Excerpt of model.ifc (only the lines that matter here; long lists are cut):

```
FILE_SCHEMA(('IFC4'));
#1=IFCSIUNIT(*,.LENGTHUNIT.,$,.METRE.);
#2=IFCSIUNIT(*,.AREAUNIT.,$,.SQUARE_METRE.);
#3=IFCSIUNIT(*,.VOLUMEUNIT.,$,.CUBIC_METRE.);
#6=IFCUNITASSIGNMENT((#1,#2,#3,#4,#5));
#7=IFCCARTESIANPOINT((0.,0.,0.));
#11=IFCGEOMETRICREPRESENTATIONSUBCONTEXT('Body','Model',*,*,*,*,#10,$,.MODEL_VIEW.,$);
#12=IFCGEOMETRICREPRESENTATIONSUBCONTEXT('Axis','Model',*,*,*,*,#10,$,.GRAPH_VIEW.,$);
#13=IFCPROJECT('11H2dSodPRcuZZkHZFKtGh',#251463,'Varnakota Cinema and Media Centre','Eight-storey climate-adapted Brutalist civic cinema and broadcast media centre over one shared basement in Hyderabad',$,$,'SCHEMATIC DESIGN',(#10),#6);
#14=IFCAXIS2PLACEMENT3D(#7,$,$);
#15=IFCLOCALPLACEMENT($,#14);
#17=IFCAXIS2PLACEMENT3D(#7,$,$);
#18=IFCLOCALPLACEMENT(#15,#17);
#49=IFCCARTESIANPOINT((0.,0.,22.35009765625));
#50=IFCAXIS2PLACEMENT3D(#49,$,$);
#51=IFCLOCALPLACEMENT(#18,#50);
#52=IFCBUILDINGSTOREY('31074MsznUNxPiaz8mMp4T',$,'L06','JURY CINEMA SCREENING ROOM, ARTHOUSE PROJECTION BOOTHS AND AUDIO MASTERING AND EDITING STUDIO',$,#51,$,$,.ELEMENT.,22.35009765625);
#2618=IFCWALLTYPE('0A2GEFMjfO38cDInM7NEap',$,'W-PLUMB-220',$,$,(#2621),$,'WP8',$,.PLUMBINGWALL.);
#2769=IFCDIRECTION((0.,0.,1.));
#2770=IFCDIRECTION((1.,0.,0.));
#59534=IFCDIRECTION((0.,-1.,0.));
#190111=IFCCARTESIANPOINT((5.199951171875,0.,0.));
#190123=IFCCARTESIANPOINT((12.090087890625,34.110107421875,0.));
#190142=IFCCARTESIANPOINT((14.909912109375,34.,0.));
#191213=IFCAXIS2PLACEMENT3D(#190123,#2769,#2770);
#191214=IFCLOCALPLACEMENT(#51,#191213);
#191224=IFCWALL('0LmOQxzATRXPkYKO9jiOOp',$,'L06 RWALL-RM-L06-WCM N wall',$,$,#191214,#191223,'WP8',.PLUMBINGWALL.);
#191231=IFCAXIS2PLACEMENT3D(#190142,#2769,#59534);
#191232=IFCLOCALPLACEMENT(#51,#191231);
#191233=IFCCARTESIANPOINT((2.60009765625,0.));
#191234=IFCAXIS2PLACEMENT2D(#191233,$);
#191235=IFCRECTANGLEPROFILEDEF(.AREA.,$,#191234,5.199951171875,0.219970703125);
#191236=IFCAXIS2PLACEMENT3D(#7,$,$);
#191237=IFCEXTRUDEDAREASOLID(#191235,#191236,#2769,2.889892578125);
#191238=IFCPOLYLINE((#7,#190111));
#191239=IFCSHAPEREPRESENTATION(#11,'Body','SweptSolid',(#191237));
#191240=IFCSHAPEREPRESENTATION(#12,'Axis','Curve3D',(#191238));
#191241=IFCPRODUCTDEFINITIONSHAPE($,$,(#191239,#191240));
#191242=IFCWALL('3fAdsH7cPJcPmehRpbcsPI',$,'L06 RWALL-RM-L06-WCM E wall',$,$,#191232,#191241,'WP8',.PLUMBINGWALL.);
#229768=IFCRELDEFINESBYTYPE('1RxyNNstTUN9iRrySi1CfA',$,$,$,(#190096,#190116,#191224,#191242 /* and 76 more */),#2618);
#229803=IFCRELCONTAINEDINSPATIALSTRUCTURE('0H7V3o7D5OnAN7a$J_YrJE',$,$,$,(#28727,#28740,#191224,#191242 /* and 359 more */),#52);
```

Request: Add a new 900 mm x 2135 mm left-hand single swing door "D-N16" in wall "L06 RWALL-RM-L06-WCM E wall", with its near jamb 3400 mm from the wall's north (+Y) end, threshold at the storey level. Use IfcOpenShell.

```python
import numpy as np
import ifcopenshell
import ifcopenshell.api.feature
import ifcopenshell.api.geometry
import ifcopenshell.api.root
import ifcopenshell.api.spatial
import ifcopenshell.geom
import ifcopenshell.util.element
import ifcopenshell.util.placement
import ifcopenshell.util.representation
import ifcopenshell.util.shape
import ifcopenshell.util.unit

model = ifcopenshell.open("model.ifc")
unit_scale = ifcopenshell.util.unit.calculate_unit_scale(model)
settings = ifcopenshell.geom.settings()


def volume(element):
    """Net volume in cubic metres, openings subtracted."""
    shape = ifcopenshell.geom.create_shape(settings, element)
    return ifcopenshell.util.shape.get_volume(shape.geometry)


wall = model.by_guid("3fAdsH7cPJcPmehRpbcsPI")
storey = ifcopenshell.util.element.get_container(wall, ifc_class="IfcBuildingStorey")
context = ifcopenshell.util.representation.get_context(model, "Model", "Body", "MODEL_VIEW")
before = volume(wall)

width, height, from_end, sill = 0.9, 2.135, 3.4, 0.0  # metres

# The wall runs along its own X axis, and the end named is its -X end.
wall_shape = ifcopenshell.geom.create_shape(settings, wall)
x, y, z = ifcopenshell.util.shape.get_vertices(wall_shape.geometry).T
start = x.min() + from_end
face, thickness = float(y.min()), float(y.max() - y.min())
wall_matrix = ifcopenshell.util.placement.get_local_placement(wall.ObjectPlacement)
level = ifcopenshell.util.placement.get_local_placement(storey.ObjectPlacement)[2, 3]


def in_wall(x, y):
    """Placement at x, y metres in the wall's axes, at sill height."""
    matrix = wall_matrix.copy()
    matrix[:, 3] = wall_matrix @ np.array([x / unit_scale, y / unit_scale, 0.0, 1.0])
    matrix[2, 3] = level + sill / unit_scale
    return matrix


# Opening: a box that overshoots both wall faces by 50 mm.
opening = ifcopenshell.api.root.create_entity(model, ifc_class="IfcOpeningElement", predefined_type="OPENING")
box = ifcopenshell.api.geometry.add_wall_representation(
    model, context=context, length=width, height=height, thickness=thickness + 0.1
)
ifcopenshell.api.geometry.assign_representation(model, product=opening, representation=box)
ifcopenshell.api.geometry.edit_object_placement(model, product=opening, matrix=in_wall(start, face - 0.05), is_si=False)
ifcopenshell.api.feature.add_feature(model, feature=opening, element=wall)

door = ifcopenshell.api.root.create_entity(model, ifc_class="IfcDoor", name="D-N16", predefined_type="DOOR")
door.OverallWidth, door.OverallHeight = width / unit_scale, height / unit_scale
door.OperationType = "SINGLE_SWING_LEFT"
body = ifcopenshell.api.geometry.add_door_representation(
    model,
    context=context,
    overall_width=door.OverallWidth,
    overall_height=door.OverallHeight,
    operation_type="SINGLE_SWING_LEFT",
    lining_properties={"LiningDepth": thickness / unit_scale, "ThresholdDepth": thickness / unit_scale},
)
ifcopenshell.api.geometry.assign_representation(model, product=door, representation=body)
ifcopenshell.api.spatial.assign_container(model, products=[door], relating_structure=storey)
ifcopenshell.api.feature.add_filling(model, opening=opening, element=door)

# The lining spans the wall, so the door starts at the wall face.
ifcopenshell.api.geometry.edit_object_placement(model, product=door, matrix=in_wall(start, face), is_si=False)

after = volume(wall)

print(f"wall volume {before:.3f} -> {after:.3f} m3")

model.write("model_edited.ifc")
```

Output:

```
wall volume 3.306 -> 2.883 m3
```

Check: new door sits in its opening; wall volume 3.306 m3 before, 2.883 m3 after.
